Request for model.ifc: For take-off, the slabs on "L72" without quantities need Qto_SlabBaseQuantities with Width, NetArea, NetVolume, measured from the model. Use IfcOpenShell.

First a look at what the model holds.

```python
import ifcopenshell
import ifcopenshell.util.element
import ifcopenshell.util.unit

model = ifcopenshell.open("model.ifc")
print(model.schema)
for unit_type in ("LENGTHUNIT", "AREAUNIT", "VOLUMEUNIT"):
    print(unit_type, ifcopenshell.util.unit.calculate_unit_scale(model, unit_type))
storey = next(s for s in model.by_type("IfcBuildingStorey") if s.Name == "L72")
slabs = [e for e in ifcopenshell.util.element.get_decomposition(storey) if e.is_a("IfcSlab")]
for e in sorted(slabs, key=lambda e: e.id()):
    print(e.id(), e.is_a(), e.Name, list(ifcopenshell.util.element.get_psets(e, qtos_only=True)), sep=" | ")
```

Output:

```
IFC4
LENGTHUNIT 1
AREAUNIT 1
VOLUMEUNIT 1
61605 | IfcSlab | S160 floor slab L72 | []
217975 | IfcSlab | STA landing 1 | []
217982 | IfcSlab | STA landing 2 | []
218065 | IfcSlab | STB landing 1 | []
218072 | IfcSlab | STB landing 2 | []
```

```python
import ifcopenshell
import ifcopenshell.api.pset
import ifcopenshell.geom
import ifcopenshell.util.element
import ifcopenshell.util.shape
import ifcopenshell.util.unit

model = ifcopenshell.open("model.ifc")
unit_scale = ifcopenshell.util.unit.calculate_unit_scale(model)
area_scale = ifcopenshell.util.unit.calculate_unit_scale(model, "AREAUNIT")
volume_scale = ifcopenshell.util.unit.calculate_unit_scale(model, "VOLUMEUNIT")
settings = ifcopenshell.geom.settings()

storey = next(s for s in model.by_type("IfcBuildingStorey") if s.Name == "L72")
slabs = [e for e in ifcopenshell.util.element.get_decomposition(storey) if e.is_a("IfcSlab")]

for e in sorted(slabs, key=lambda e: e.id()):
    if ifcopenshell.util.element.get_psets(e, qtos_only=True, should_inherit=False):
        continue
    # Geometry comes back in metres, in the element's own axes.
    shape = ifcopenshell.geom.create_shape(settings, e)
    values = {
        "Width": ifcopenshell.util.shape.get_z(shape.geometry) / unit_scale,
        "NetArea": ifcopenshell.util.shape.get_footprint_area(shape.geometry) / area_scale,
        "NetVolume": ifcopenshell.util.shape.get_volume(shape.geometry) / volume_scale,
    }
    qto = ifcopenshell.api.pset.add_qto(model, product=e, name="Qto_SlabBaseQuantities")
    ifcopenshell.api.pset.edit_qto(model, qto=qto, properties=values)
    print(e.id(), {k: round(v, 3) for k, v in values.items()})

model.write("model_updated.ifc")
```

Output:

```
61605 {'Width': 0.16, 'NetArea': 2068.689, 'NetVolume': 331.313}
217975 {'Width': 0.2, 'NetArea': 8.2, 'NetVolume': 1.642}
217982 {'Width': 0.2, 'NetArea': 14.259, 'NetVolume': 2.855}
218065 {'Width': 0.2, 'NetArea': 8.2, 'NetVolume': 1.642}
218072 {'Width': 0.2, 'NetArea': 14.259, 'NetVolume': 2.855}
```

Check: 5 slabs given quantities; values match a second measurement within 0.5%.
